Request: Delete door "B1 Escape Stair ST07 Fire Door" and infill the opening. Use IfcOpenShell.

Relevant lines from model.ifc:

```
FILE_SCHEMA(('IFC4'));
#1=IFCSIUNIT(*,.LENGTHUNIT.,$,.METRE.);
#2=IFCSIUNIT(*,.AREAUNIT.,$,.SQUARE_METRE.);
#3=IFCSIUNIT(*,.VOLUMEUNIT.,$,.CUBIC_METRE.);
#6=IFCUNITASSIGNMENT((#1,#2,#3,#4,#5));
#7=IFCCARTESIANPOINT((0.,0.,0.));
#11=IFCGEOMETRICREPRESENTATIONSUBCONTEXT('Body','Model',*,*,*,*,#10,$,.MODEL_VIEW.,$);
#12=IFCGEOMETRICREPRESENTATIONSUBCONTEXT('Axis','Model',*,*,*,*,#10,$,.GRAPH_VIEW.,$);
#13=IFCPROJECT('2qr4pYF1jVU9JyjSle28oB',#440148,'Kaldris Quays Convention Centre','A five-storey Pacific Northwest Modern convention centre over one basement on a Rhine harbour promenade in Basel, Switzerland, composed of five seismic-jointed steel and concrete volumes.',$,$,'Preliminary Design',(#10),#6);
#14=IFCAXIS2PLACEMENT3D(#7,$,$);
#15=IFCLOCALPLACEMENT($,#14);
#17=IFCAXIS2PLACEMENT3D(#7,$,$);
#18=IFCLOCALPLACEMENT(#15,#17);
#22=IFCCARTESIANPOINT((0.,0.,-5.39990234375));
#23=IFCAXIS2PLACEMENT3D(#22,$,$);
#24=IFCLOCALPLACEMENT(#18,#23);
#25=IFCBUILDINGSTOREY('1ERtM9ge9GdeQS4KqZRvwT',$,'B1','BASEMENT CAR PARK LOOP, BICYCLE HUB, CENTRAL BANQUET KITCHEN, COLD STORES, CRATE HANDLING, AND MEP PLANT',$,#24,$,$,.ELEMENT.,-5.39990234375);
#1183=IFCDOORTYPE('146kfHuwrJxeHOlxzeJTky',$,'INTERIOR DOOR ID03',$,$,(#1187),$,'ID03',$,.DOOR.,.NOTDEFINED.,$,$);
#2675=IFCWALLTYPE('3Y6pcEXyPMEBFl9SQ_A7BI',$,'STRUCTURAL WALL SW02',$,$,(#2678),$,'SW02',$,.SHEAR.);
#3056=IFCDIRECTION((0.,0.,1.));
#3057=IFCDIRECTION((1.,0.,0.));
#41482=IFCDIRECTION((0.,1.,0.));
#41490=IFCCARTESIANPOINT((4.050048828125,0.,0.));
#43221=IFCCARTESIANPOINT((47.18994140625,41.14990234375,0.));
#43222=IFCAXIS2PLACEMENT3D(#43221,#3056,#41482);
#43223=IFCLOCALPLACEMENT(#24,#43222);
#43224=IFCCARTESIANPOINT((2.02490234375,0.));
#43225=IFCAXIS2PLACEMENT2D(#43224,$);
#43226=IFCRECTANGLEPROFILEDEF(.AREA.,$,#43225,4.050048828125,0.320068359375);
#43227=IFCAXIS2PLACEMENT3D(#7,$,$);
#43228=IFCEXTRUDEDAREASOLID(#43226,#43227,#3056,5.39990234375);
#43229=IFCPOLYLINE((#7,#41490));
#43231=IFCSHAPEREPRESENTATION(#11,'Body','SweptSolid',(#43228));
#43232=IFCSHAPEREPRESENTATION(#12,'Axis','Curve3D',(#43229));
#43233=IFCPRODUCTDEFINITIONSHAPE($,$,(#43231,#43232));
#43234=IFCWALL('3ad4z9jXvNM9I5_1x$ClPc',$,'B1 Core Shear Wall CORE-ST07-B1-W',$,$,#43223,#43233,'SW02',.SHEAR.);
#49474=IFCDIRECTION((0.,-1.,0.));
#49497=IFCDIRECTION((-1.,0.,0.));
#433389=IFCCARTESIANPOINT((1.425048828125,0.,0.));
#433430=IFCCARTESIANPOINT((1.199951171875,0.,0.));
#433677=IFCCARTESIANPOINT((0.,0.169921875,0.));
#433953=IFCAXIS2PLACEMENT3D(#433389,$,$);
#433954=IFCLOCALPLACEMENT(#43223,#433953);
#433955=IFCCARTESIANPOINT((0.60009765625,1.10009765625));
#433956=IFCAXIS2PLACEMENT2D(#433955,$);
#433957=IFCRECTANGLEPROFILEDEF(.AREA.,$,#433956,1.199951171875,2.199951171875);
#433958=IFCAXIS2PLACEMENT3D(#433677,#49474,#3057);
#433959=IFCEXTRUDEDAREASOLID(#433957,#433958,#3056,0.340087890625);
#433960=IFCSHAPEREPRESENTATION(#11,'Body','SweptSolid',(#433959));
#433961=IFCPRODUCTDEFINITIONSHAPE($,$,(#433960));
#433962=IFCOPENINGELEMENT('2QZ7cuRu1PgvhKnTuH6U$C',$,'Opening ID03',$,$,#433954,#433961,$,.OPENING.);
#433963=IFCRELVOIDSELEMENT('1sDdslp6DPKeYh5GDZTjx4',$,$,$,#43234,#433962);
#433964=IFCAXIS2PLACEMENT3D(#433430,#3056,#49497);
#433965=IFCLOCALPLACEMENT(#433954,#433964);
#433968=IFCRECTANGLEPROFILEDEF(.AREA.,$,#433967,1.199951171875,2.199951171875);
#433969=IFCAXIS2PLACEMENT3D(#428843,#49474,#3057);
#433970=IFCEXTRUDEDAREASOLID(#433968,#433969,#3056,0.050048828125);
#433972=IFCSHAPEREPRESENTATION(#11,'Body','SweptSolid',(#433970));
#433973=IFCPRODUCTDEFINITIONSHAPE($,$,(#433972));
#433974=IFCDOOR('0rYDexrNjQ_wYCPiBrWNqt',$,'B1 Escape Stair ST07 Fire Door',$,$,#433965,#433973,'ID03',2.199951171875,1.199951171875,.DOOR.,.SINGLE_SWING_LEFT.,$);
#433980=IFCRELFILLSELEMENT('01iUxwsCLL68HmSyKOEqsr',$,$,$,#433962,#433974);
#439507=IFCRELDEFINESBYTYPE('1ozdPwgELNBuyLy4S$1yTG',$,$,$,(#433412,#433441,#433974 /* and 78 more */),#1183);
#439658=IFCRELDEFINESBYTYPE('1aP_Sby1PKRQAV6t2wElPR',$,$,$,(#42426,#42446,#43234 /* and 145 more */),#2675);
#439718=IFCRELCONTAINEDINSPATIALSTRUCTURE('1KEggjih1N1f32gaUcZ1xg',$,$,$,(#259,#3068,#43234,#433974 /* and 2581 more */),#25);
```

```python
import ifcopenshell
import ifcopenshell.api.feature
import ifcopenshell.api.root
import ifcopenshell.geom
import ifcopenshell.util.shape

model = ifcopenshell.open("model.ifc")
settings = ifcopenshell.geom.settings()


def volume(element):
    """Net volume in cubic metres, openings subtracted."""
    shape = ifcopenshell.geom.create_shape(settings, element)
    return ifcopenshell.util.shape.get_volume(shape.geometry)


door = model.by_id(433974)
opening = door.FillsVoids[0].RelatingOpeningElement
wall = opening.VoidsElements[0].RelatingBuildingElement
before = volume(wall)

ifcopenshell.api.root.remove_product(model, product=door)
ifcopenshell.api.feature.remove_feature(model, feature=opening)

after = volume(wall)

print(f"wall volume {before:.3f} -> {after:.3f} m3")

model.write("model-out.ifc")
```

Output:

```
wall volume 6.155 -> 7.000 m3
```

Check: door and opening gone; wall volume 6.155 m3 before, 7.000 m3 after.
